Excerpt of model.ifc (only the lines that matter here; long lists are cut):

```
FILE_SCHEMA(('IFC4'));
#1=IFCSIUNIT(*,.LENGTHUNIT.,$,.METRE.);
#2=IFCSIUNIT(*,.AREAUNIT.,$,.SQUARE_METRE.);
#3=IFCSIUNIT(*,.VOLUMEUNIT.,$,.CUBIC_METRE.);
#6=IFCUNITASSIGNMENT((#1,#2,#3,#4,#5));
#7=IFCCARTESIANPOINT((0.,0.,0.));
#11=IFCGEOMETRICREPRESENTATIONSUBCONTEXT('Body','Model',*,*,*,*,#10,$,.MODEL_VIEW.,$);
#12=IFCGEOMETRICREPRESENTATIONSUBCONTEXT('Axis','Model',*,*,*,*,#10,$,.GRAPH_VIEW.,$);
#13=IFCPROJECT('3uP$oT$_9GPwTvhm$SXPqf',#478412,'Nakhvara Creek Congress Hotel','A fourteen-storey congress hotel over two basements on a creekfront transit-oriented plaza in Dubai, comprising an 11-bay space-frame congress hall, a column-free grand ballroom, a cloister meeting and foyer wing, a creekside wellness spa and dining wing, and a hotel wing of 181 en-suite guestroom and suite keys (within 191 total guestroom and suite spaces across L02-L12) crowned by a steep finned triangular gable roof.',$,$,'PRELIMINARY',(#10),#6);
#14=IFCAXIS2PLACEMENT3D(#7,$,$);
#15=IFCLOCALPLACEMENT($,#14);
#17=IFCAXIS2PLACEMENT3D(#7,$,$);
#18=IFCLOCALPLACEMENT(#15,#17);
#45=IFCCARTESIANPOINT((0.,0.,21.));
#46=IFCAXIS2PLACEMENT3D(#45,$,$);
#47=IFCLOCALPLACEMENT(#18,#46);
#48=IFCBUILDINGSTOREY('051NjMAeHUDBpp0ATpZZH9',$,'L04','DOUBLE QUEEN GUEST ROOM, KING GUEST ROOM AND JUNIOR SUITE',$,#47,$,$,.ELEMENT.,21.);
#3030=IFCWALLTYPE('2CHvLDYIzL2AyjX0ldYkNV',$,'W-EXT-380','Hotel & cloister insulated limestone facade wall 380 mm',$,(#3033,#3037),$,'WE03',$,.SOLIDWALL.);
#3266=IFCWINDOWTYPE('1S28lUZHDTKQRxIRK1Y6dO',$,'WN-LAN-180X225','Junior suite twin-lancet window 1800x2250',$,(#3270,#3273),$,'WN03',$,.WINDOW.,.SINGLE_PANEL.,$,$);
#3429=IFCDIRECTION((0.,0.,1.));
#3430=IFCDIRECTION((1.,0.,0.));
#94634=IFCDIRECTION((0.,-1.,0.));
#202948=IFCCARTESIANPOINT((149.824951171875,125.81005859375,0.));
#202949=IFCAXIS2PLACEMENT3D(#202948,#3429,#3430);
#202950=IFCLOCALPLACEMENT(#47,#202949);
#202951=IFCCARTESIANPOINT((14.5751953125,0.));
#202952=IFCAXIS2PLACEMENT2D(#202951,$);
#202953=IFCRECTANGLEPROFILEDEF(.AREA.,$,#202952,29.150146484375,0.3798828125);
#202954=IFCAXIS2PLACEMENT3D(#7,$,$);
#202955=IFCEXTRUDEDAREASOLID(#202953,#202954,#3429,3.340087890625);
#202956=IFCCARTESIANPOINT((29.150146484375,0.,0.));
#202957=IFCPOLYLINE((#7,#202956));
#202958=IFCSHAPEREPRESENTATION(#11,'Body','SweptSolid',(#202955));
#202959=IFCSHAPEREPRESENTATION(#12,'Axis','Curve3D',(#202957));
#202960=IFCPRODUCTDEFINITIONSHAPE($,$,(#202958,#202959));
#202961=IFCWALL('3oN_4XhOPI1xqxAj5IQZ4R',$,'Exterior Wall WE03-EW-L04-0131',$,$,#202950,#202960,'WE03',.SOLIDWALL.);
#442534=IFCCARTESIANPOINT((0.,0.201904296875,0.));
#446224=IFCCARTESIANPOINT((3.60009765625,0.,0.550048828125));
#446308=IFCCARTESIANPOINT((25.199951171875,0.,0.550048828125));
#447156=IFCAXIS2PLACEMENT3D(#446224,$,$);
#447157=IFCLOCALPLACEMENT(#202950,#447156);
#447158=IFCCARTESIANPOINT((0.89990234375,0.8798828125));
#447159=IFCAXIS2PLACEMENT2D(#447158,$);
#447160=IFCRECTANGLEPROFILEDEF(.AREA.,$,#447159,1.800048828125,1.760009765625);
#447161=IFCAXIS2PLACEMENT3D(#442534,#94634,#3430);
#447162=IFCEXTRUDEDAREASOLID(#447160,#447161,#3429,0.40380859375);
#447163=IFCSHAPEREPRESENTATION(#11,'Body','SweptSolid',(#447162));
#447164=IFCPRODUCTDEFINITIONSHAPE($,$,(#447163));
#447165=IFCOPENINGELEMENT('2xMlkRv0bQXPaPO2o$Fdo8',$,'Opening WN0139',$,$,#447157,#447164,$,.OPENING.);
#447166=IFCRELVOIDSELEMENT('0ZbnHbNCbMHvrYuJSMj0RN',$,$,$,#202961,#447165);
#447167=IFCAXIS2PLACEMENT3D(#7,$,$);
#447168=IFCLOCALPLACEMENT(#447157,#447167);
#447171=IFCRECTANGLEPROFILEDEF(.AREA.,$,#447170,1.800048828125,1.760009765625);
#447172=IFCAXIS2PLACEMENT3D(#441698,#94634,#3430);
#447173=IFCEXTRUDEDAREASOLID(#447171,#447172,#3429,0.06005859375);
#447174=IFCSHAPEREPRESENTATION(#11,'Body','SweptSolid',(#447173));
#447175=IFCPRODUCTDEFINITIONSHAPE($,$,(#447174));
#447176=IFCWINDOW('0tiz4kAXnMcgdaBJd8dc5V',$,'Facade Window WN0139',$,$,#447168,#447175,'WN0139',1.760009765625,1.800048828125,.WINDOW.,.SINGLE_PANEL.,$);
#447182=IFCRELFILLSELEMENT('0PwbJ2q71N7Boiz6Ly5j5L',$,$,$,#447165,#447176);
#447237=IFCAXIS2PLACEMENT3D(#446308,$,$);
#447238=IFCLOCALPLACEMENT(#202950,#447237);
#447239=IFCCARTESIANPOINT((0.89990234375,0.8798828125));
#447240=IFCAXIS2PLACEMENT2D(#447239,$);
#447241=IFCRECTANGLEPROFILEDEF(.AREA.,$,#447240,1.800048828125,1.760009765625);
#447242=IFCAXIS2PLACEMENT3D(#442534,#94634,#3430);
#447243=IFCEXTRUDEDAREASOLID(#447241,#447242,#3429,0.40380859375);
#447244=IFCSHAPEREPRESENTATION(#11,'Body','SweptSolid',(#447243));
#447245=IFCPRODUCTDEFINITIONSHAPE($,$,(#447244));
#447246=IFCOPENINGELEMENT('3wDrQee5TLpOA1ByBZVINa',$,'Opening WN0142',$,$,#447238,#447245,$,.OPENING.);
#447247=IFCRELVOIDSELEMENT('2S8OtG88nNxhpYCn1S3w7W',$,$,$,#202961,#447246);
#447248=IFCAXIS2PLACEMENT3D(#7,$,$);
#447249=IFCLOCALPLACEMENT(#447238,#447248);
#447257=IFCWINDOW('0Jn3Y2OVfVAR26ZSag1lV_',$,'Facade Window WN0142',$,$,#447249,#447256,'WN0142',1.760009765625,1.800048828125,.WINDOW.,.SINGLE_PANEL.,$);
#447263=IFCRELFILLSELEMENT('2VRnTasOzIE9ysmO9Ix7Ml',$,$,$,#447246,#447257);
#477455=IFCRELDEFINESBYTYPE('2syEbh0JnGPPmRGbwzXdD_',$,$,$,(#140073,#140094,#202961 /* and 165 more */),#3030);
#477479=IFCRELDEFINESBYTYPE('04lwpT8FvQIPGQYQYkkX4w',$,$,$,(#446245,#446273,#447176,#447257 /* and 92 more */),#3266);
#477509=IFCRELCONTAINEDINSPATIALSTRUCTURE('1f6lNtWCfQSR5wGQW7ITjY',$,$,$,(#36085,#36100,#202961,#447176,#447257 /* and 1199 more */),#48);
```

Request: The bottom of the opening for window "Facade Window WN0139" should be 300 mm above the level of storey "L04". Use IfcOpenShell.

```python
import numpy as np
import ifcopenshell
import ifcopenshell.api.geometry
import ifcopenshell.geom
import ifcopenshell.util.element
import ifcopenshell.util.placement
import ifcopenshell.util.shape
import ifcopenshell.util.unit

model = ifcopenshell.open("model.ifc")
unit_scale = ifcopenshell.util.unit.calculate_unit_scale(model)

window = model.by_guid("0tiz4kAXnMcgdaBJd8dc5V")
opening = window.FillsVoids[0].RelatingOpeningElement
storey = ifcopenshell.util.element.get_container(window, ifc_class="IfcBuildingStorey")
level = ifcopenshell.util.placement.get_local_placement(storey.ObjectPlacement)[2, 3]

# The opening's origin need not be at the sill, so measure its lowest point.
shape = ifcopenshell.geom.create_shape(ifcopenshell.geom.settings(), opening)
bottom = ifcopenshell.util.shape.get_shape_bottom_elevation(shape, shape.geometry) / unit_scale
dz = level + 0.3 / unit_scale - bottom

shift = np.array([0.0, 0.0, dz])
# The window is placed relative to its opening, so it follows when the opening moves.
matrix = ifcopenshell.util.placement.get_local_placement(opening.ObjectPlacement)
matrix[:3, 3] += shift
ifcopenshell.api.geometry.edit_object_placement(
    model, product=opening, matrix=matrix, is_si=False, should_transform_children=True
)

print(f"moved by {dz * unit_scale:+.3f} m")

model.write("model_v2.ifc")
```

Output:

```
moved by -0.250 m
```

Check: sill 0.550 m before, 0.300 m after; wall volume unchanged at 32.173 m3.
